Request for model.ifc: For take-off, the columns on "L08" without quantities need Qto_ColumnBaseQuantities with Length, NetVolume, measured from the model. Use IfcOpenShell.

First a look at what the model holds.

```python
import ifcopenshell
import ifcopenshell.util.element
import ifcopenshell.util.unit

model = ifcopenshell.open("model.ifc")
print(model.schema)
for unit_type in ("LENGTHUNIT", "AREAUNIT", "VOLUMEUNIT"):
    print(unit_type, ifcopenshell.util.unit.calculate_unit_scale(model, unit_type))
storey = next(s for s in model.by_type("IfcBuildingStorey") if s.Name == "L08")
columns = [e for e in ifcopenshell.util.element.get_decomposition(storey) if e.is_a("IfcColumn")]
for e in sorted(columns, key=lambda e: e.id()):
    print(e.id(), e.is_a(), e.Name, list(ifcopenshell.util.element.get_psets(e, qtos_only=True)), sep=" | ")
```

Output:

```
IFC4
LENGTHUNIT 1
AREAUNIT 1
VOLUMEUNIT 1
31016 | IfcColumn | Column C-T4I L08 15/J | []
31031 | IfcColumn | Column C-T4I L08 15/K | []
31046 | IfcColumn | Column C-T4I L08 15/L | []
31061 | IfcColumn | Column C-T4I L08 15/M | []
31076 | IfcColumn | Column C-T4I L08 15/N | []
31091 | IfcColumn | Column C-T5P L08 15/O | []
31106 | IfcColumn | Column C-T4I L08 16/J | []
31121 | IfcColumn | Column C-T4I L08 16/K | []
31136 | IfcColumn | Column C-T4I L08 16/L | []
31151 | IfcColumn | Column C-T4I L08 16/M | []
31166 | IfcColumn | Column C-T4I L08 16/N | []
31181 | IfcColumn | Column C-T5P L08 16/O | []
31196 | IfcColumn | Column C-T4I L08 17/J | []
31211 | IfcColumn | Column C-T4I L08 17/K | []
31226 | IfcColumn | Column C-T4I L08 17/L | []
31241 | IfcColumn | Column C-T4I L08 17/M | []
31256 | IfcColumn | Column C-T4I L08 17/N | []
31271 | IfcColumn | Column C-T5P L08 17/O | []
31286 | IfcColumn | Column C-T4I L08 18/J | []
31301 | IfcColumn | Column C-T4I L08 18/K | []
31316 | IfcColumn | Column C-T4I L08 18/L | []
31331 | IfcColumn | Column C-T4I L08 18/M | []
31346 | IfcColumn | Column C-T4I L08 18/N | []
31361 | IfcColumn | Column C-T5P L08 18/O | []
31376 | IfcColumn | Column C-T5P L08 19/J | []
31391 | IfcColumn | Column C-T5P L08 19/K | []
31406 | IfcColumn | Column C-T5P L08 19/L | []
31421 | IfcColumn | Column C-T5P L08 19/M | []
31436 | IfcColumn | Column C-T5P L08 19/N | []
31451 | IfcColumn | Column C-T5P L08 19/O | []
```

```python
import ifcopenshell
import ifcopenshell.api.pset
import ifcopenshell.geom
import ifcopenshell.util.element
import ifcopenshell.util.shape
import ifcopenshell.util.unit

model = ifcopenshell.open("model.ifc")
unit_scale = ifcopenshell.util.unit.calculate_unit_scale(model)
volume_scale = ifcopenshell.util.unit.calculate_unit_scale(model, "VOLUMEUNIT")
settings = ifcopenshell.geom.settings()

storey = next(s for s in model.by_type("IfcBuildingStorey") if s.Name == "L08")
columns = [e for e in ifcopenshell.util.element.get_decomposition(storey) if e.is_a("IfcColumn")]

for e in sorted(columns, key=lambda e: e.id()):
    if ifcopenshell.util.element.get_psets(e, qtos_only=True, should_inherit=False):
        continue
    # Geometry comes back in metres, in the element's own axes.
    shape = ifcopenshell.geom.create_shape(settings, e)
    values = {
        "Length": ifcopenshell.util.shape.get_z(shape.geometry) / unit_scale,
        "NetVolume": ifcopenshell.util.shape.get_volume(shape.geometry) / volume_scale,
    }
    qto = ifcopenshell.api.pset.add_qto(model, product=e, name="Qto_ColumnBaseQuantities")
    ifcopenshell.api.pset.edit_qto(model, qto=qto, properties=values)
    print(e.id(), {k: round(v, 3) for k, v in values.items()})

model.write("model_edited.ifc")
```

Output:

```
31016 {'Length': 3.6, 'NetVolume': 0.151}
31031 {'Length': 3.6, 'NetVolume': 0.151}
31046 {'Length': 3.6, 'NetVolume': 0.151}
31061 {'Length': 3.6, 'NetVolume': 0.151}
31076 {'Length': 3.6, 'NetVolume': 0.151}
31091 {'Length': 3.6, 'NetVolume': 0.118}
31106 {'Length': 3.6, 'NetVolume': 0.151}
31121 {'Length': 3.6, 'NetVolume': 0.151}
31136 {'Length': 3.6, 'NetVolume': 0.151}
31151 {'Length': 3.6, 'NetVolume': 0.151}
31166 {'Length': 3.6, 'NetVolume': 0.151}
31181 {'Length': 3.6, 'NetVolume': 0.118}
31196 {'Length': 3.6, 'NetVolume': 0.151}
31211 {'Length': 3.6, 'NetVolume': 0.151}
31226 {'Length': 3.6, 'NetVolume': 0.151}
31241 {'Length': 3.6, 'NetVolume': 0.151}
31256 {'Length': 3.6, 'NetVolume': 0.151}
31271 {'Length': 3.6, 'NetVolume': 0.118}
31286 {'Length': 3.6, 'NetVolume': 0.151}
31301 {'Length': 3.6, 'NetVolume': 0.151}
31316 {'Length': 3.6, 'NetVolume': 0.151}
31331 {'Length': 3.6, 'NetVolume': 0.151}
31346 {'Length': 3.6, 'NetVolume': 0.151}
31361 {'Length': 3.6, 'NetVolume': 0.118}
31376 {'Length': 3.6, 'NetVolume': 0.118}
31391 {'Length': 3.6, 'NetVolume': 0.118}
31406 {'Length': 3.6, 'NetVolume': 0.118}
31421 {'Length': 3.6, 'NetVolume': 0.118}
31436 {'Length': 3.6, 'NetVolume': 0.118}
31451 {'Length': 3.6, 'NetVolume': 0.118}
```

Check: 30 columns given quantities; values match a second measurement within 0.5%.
